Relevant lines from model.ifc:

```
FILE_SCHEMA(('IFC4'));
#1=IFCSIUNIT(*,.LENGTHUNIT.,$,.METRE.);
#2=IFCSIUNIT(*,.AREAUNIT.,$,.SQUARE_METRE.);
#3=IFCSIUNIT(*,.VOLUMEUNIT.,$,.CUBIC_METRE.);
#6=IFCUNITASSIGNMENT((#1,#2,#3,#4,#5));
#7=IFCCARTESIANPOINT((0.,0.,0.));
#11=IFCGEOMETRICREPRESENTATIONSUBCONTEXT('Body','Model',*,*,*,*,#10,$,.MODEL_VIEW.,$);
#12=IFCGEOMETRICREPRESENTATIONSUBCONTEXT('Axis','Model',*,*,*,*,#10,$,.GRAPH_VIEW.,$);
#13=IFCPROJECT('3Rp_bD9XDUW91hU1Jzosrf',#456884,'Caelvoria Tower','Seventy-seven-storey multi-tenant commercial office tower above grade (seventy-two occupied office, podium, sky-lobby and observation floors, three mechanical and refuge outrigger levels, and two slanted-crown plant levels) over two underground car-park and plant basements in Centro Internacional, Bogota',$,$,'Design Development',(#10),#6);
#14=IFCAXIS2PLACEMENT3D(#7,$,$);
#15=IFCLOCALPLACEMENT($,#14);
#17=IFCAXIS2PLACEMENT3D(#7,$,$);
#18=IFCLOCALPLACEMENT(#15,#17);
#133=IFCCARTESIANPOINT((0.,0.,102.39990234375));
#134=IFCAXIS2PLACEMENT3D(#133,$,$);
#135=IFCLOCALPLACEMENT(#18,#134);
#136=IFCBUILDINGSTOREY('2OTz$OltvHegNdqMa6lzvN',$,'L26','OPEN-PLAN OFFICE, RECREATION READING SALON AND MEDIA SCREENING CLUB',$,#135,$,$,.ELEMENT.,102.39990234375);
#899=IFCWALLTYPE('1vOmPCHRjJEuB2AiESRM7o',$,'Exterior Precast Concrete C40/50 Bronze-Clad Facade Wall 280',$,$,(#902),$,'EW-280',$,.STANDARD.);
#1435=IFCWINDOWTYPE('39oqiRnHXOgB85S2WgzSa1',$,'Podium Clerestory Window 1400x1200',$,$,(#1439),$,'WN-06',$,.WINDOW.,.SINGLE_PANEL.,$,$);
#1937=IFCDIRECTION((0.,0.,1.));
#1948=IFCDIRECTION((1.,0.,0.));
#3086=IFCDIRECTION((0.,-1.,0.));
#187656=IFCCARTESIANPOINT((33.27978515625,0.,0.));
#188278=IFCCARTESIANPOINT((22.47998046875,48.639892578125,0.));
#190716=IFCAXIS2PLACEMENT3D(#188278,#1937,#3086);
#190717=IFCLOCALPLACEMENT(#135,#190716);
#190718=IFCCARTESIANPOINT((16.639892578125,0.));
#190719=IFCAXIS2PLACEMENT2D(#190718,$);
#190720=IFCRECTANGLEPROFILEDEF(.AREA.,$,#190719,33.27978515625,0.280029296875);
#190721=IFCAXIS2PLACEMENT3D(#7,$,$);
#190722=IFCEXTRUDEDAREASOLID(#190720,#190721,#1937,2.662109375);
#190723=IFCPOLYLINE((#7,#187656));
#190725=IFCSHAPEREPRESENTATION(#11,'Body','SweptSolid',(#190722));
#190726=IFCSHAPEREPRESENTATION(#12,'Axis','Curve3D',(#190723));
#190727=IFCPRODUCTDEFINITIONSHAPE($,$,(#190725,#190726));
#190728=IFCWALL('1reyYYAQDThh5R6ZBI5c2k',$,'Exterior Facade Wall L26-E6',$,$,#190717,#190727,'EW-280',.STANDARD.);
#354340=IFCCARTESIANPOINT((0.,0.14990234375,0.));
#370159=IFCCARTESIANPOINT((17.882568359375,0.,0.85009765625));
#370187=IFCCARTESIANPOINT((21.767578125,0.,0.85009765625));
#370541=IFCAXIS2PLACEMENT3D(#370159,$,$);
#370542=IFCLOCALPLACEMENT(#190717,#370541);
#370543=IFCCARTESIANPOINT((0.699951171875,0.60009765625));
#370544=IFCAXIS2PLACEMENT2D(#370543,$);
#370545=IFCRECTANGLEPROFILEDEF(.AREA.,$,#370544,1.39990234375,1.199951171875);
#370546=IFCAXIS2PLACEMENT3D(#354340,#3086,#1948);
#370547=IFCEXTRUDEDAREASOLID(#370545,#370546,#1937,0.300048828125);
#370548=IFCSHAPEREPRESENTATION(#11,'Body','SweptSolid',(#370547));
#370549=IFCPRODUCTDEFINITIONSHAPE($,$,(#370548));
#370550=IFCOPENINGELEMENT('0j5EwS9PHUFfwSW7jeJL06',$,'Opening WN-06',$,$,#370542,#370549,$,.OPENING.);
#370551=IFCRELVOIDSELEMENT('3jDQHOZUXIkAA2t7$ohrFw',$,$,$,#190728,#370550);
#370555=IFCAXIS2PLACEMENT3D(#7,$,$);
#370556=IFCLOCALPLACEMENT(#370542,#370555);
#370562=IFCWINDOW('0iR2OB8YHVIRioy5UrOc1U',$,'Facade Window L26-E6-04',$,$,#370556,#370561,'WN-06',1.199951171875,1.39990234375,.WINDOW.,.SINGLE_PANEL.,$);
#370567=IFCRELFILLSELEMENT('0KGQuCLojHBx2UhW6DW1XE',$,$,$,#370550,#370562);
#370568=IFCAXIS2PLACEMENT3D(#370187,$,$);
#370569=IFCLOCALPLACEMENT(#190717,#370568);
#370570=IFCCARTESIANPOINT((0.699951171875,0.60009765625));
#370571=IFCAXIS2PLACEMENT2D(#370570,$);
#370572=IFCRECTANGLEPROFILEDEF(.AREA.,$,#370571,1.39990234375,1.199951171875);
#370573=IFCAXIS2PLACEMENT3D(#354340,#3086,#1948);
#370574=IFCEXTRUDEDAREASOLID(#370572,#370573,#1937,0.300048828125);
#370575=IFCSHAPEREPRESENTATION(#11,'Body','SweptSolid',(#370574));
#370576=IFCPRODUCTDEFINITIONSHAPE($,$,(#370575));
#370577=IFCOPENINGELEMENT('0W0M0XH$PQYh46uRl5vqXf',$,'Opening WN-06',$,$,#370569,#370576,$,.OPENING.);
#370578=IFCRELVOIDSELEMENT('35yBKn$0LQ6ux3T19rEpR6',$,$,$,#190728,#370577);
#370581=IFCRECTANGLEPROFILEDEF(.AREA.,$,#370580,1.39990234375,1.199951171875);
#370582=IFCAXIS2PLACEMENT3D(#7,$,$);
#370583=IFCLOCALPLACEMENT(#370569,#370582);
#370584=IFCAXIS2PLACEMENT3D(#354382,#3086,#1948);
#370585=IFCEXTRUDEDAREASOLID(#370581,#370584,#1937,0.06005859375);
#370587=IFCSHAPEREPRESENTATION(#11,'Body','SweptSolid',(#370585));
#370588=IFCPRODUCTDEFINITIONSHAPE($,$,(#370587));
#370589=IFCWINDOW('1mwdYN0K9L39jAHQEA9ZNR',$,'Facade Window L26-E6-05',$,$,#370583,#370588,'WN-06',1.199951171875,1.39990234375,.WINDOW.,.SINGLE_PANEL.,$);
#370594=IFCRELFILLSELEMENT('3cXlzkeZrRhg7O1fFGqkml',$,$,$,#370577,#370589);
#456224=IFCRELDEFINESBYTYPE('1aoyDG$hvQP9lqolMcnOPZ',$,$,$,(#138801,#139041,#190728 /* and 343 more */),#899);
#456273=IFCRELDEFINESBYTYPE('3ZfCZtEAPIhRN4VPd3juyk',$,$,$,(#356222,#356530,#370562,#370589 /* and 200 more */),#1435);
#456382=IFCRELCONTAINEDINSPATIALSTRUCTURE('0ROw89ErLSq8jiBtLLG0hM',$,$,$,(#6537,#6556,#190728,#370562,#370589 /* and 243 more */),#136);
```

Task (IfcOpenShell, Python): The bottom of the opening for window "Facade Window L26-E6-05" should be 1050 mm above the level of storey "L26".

```python
import numpy as np
import ifcopenshell
import ifcopenshell.api.geometry
import ifcopenshell.geom
import ifcopenshell.util.element
import ifcopenshell.util.placement
import ifcopenshell.util.shape
import ifcopenshell.util.unit

model = ifcopenshell.open("model.ifc")
unit_scale = ifcopenshell.util.unit.calculate_unit_scale(model)

window = model.by_guid("1mwdYN0K9L39jAHQEA9ZNR")
opening = window.FillsVoids[0].RelatingOpeningElement
storey = ifcopenshell.util.element.get_container(window, ifc_class="IfcBuildingStorey")
level = ifcopenshell.util.placement.get_local_placement(storey.ObjectPlacement)[2, 3]

# The opening's origin need not be at the sill, so measure its lowest point.
shape = ifcopenshell.geom.create_shape(ifcopenshell.geom.settings(), opening)
bottom = ifcopenshell.util.shape.get_shape_bottom_elevation(shape, shape.geometry) / unit_scale
dz = level + 1.05 / unit_scale - bottom

shift = np.array([0.0, 0.0, dz])
# The window is placed relative to its opening, so it follows when the opening moves.
matrix = ifcopenshell.util.placement.get_local_placement(opening.ObjectPlacement)
matrix[:3, 3] += shift
ifcopenshell.api.geometry.edit_object_placement(
    model, product=opening, matrix=matrix, is_si=False, should_transform_children=True
)

print(f"moved by {dz * unit_scale:+.3f} m")

model.write("model-out.ifc")
```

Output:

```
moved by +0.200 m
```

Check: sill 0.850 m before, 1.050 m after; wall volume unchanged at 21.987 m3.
